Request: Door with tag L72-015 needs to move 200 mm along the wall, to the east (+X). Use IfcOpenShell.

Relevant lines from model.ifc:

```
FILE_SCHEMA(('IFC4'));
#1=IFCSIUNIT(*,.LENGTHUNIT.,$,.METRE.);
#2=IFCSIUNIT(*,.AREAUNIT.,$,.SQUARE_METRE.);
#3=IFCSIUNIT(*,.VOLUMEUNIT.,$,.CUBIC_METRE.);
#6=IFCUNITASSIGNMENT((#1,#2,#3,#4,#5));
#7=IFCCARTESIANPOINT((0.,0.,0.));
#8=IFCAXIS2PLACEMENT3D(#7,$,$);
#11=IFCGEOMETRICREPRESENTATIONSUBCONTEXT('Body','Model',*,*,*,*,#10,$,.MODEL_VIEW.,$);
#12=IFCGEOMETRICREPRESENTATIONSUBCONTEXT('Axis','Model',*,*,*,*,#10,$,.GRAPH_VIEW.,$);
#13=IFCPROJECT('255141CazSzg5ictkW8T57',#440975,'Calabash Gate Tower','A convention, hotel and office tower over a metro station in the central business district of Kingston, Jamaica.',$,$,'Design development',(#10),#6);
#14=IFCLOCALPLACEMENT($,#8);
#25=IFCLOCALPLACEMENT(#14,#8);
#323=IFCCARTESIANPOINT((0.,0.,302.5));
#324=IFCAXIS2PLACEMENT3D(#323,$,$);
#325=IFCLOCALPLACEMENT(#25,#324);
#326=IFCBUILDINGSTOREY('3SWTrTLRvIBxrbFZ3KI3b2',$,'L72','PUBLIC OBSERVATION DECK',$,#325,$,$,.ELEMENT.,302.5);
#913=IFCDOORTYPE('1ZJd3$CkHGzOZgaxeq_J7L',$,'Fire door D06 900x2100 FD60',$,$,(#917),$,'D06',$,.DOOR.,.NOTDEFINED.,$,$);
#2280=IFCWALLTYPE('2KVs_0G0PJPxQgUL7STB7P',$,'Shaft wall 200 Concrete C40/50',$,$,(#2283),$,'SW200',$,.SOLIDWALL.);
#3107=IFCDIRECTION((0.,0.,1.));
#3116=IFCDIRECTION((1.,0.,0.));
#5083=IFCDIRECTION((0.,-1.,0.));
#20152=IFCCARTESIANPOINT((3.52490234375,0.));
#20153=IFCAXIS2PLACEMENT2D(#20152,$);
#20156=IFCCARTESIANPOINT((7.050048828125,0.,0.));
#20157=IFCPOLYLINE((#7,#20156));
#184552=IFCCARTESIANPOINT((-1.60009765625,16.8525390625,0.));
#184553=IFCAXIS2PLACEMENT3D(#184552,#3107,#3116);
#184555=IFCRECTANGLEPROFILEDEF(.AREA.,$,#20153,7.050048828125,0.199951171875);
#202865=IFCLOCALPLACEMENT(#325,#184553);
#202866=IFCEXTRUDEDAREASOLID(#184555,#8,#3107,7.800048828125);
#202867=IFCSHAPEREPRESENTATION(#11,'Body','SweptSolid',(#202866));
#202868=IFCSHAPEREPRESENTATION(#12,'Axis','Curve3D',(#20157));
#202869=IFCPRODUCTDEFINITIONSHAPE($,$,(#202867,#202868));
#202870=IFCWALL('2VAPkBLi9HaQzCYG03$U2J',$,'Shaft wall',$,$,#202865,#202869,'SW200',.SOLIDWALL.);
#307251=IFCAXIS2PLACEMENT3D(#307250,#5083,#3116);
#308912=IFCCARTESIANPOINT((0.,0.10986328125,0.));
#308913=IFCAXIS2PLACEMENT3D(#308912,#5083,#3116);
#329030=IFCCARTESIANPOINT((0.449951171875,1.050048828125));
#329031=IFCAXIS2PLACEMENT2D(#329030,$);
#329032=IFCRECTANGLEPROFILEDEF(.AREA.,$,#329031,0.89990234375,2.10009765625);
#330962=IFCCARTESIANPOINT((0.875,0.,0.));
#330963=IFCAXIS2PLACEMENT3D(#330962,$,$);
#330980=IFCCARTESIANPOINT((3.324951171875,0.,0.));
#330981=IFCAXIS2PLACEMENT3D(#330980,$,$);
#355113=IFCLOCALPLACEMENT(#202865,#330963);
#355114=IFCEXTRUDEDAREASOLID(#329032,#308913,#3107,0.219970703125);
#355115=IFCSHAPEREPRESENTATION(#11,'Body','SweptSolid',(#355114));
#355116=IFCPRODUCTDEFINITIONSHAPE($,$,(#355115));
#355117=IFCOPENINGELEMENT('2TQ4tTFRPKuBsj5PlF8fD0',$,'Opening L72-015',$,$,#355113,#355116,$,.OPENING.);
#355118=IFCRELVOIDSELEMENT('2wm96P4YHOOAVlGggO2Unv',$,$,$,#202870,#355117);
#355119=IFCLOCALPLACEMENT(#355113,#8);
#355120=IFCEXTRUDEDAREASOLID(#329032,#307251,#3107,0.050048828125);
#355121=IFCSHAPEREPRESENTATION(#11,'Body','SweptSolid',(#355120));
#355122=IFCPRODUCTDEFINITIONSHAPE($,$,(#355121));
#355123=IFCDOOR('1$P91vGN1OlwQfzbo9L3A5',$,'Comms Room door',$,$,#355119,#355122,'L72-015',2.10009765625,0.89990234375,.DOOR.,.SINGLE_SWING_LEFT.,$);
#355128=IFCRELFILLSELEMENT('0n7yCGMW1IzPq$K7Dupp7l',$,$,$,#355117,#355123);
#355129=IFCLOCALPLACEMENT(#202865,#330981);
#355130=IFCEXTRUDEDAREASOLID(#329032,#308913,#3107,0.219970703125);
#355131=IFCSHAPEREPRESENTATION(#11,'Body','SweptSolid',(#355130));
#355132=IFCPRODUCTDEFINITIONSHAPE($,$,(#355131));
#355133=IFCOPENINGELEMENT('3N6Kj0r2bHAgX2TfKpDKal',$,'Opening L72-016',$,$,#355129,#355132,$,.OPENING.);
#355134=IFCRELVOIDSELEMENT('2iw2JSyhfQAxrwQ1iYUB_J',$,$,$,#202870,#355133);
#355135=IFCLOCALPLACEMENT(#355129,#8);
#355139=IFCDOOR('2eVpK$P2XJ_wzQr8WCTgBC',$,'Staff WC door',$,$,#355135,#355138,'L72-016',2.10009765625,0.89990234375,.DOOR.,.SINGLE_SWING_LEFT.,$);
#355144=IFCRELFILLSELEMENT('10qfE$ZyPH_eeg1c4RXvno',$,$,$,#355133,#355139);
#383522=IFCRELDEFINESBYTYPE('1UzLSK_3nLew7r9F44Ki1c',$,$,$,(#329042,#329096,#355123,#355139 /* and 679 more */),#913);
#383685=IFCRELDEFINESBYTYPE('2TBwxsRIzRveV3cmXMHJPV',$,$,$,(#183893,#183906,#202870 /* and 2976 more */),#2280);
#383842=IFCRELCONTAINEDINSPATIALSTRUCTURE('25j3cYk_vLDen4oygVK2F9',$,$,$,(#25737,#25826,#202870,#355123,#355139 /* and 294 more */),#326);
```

```python
import ifcopenshell
import ifcopenshell.api.geometry
import ifcopenshell.util.placement

model = ifcopenshell.open("model.ifc")

door = model.by_guid("1$P91vGN1OlwQfzbo9L3A5")
opening = door.FillsVoids[0].RelatingOpeningElement
wall = opening.VoidsElements[0].RelatingBuildingElement

wall_matrix = ifcopenshell.util.placement.get_local_placement(wall.ObjectPlacement)
shift = wall_matrix[:3, 0] * 0.2
before = ifcopenshell.util.placement.get_local_placement(door.ObjectPlacement)[:3, 3].copy()

# The door is placed relative to its opening, so it follows when the opening moves.
matrix = ifcopenshell.util.placement.get_local_placement(opening.ObjectPlacement)
matrix[:3, 3] += shift
ifcopenshell.api.geometry.edit_object_placement(
    model, product=opening, matrix=matrix, is_si=False, should_transform_children=True
)

after = ifcopenshell.util.placement.get_local_placement(door.ObjectPlacement)[:3, 3]
print("door moved by", (after - before).round(3) + 0.0)

model.write("model_edited.ifc")
```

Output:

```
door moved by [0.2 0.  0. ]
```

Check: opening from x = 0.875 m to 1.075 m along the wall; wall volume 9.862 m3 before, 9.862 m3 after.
